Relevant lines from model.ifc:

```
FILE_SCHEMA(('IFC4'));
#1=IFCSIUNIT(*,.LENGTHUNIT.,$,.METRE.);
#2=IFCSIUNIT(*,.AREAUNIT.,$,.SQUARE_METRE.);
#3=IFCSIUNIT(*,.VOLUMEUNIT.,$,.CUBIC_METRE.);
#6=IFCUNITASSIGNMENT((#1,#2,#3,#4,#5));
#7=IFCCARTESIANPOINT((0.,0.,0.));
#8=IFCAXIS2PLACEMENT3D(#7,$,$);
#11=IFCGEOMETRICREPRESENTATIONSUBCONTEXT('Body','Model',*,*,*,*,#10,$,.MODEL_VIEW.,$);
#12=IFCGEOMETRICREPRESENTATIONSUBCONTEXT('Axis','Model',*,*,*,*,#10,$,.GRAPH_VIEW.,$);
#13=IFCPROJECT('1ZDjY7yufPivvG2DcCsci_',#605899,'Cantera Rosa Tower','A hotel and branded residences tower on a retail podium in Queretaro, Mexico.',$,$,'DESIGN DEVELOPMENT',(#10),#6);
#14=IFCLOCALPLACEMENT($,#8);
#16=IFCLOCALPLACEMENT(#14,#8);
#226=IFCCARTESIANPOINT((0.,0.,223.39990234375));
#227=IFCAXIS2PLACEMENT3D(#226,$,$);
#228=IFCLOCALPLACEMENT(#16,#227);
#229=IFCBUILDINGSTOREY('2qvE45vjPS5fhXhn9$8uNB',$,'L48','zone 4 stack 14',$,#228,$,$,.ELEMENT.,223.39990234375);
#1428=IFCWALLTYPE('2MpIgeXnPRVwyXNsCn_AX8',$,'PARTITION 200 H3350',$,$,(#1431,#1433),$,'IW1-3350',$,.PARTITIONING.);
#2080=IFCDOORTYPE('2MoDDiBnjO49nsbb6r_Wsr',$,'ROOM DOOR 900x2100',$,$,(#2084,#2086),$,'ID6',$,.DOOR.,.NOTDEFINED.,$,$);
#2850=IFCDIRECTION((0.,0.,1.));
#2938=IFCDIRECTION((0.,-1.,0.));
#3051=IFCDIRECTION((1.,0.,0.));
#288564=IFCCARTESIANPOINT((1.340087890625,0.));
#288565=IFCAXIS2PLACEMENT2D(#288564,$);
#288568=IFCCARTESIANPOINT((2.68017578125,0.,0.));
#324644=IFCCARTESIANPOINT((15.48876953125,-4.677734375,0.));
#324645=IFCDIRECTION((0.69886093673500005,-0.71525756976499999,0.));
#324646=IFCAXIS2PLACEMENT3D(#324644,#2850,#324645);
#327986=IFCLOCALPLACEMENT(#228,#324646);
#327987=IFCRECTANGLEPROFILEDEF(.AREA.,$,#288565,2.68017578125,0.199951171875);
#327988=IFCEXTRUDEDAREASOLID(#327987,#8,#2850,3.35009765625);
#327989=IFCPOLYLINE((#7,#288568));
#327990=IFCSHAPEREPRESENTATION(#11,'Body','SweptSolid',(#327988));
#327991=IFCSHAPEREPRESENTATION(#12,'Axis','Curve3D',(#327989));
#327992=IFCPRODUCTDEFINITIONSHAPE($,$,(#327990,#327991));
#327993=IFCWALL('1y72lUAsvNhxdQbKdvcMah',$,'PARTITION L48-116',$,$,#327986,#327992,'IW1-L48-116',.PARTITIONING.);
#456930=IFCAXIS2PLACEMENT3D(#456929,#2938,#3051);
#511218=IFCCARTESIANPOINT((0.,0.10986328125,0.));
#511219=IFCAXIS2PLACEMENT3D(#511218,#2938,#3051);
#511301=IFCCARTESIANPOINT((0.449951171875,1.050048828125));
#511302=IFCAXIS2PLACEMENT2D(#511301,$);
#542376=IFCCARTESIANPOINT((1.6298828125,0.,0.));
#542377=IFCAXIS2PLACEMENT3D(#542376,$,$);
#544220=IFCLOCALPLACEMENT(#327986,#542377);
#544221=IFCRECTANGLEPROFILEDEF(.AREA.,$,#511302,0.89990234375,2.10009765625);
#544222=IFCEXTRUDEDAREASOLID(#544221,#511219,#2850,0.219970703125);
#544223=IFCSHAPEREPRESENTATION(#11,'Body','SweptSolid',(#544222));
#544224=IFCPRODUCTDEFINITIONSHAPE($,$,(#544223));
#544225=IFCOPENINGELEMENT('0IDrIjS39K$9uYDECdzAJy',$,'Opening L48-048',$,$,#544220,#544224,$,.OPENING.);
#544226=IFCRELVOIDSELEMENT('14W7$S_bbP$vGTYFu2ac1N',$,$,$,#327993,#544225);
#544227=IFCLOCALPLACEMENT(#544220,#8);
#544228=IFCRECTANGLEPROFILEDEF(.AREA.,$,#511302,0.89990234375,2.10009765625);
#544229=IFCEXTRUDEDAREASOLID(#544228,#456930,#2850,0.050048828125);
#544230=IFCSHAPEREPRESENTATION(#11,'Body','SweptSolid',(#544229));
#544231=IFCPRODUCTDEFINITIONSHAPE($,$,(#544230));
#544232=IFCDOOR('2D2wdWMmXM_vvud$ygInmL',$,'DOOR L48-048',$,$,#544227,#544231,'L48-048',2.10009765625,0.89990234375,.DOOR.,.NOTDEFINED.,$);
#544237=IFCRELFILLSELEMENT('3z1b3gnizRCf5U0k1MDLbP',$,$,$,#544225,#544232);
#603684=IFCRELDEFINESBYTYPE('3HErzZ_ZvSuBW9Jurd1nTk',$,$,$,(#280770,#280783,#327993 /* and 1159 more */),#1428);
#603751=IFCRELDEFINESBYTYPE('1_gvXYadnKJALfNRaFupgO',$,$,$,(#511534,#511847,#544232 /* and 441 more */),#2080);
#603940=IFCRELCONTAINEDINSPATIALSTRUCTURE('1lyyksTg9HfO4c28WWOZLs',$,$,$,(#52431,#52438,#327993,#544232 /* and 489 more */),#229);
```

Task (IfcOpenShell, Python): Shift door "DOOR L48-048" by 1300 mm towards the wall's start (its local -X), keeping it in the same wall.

```python
import ifcopenshell
import ifcopenshell.api.geometry
import ifcopenshell.util.placement

model = ifcopenshell.open("model.ifc")

door = model.by_guid("2D2wdWMmXM_vvud$ygInmL")
opening = door.FillsVoids[0].RelatingOpeningElement
wall = opening.VoidsElements[0].RelatingBuildingElement

wall_matrix = ifcopenshell.util.placement.get_local_placement(wall.ObjectPlacement)
shift = wall_matrix[:3, 0] * -1.3
before = ifcopenshell.util.placement.get_local_placement(door.ObjectPlacement)[:3, 3].copy()

# The door is placed relative to its opening, so it follows when the opening moves.
matrix = ifcopenshell.util.placement.get_local_placement(opening.ObjectPlacement)
matrix[:3, 3] += shift
ifcopenshell.api.geometry.edit_object_placement(
    model, product=opening, matrix=matrix, is_si=False, should_transform_children=True
)

after = ifcopenshell.util.placement.get_local_placement(door.ObjectPlacement)[:3, 3]
print("door moved by", (after - before).round(3) + 0.0)

model.write("model_rev.ifc")
```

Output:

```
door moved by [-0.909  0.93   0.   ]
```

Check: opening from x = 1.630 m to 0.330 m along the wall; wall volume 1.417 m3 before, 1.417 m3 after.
